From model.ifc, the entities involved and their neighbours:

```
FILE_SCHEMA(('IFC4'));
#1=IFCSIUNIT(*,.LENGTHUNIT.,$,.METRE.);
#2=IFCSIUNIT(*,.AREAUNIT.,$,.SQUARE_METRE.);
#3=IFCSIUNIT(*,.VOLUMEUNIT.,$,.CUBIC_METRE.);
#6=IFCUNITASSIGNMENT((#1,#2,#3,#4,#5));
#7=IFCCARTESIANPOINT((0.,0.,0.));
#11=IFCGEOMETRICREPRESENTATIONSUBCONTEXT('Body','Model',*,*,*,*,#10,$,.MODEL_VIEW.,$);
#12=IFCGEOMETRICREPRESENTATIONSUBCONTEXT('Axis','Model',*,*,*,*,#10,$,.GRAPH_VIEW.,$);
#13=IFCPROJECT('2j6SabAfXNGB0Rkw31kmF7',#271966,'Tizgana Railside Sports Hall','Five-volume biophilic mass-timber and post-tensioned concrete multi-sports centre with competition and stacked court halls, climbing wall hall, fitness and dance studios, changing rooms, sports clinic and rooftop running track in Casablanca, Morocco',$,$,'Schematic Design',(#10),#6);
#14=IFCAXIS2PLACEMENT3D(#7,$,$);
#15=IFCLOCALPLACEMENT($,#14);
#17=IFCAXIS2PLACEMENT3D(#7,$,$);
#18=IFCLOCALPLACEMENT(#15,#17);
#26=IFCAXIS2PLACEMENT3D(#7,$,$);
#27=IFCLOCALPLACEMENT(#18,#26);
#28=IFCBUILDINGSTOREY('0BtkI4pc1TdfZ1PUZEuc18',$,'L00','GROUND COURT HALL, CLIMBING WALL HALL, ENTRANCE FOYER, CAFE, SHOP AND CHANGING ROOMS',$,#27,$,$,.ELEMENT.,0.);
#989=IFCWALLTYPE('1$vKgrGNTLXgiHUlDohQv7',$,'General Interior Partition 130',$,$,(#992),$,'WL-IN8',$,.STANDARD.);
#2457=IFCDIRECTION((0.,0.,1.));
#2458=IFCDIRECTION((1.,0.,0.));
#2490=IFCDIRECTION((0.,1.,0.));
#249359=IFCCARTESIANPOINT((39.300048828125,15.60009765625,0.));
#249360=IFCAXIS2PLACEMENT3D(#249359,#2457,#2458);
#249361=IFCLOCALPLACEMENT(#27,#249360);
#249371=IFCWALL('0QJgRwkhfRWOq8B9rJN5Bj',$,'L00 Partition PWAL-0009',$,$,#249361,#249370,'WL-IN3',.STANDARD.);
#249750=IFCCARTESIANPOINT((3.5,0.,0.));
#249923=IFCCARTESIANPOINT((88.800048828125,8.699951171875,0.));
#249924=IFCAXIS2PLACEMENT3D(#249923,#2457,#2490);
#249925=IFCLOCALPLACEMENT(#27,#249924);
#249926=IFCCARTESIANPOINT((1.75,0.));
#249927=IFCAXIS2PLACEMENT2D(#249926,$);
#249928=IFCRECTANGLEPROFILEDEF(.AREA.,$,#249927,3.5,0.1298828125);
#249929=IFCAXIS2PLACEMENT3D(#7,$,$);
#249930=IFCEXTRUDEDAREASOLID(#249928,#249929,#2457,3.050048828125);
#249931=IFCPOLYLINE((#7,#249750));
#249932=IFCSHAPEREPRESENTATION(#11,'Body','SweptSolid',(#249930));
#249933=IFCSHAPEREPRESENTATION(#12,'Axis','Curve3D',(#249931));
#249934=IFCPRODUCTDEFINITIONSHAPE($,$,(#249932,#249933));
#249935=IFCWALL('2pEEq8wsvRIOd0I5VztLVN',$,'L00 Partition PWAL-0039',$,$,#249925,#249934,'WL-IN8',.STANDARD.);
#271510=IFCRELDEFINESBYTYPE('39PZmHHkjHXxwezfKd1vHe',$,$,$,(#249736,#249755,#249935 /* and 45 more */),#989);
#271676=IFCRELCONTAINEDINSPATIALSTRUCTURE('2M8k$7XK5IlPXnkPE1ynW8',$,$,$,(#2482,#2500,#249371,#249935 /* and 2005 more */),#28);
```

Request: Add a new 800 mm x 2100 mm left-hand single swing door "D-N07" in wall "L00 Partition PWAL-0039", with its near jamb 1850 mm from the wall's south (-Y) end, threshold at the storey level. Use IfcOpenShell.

```python
import numpy as np
import ifcopenshell
import ifcopenshell.api.feature
import ifcopenshell.api.geometry
import ifcopenshell.api.root
import ifcopenshell.api.spatial
import ifcopenshell.geom
import ifcopenshell.util.element
import ifcopenshell.util.placement
import ifcopenshell.util.representation
import ifcopenshell.util.shape
import ifcopenshell.util.unit

model = ifcopenshell.open("model.ifc")
unit_scale = ifcopenshell.util.unit.calculate_unit_scale(model)
settings = ifcopenshell.geom.settings()


def volume(element):
    """Net volume in cubic metres, openings subtracted."""
    shape = ifcopenshell.geom.create_shape(settings, element)
    return ifcopenshell.util.shape.get_volume(shape.geometry)


wall = model.by_guid("2pEEq8wsvRIOd0I5VztLVN")
storey = ifcopenshell.util.element.get_container(wall, ifc_class="IfcBuildingStorey")
context = ifcopenshell.util.representation.get_context(model, "Model", "Body", "MODEL_VIEW")
before = volume(wall)

width, height, from_end, sill = 0.8, 2.1, 1.85, 0.0  # metres

# The wall runs along its own X axis, and the end named is its -X end.
wall_shape = ifcopenshell.geom.create_shape(settings, wall)
x, y, z = ifcopenshell.util.shape.get_vertices(wall_shape.geometry).T
start = x.min() + from_end
face, thickness = float(y.min()), float(y.max() - y.min())
wall_matrix = ifcopenshell.util.placement.get_local_placement(wall.ObjectPlacement)
level = ifcopenshell.util.placement.get_local_placement(storey.ObjectPlacement)[2, 3]


def in_wall(x, y):
    """Placement at x, y metres in the wall's axes, at sill height."""
    matrix = wall_matrix.copy()
    matrix[:, 3] = wall_matrix @ np.array([x / unit_scale, y / unit_scale, 0.0, 1.0])
    matrix[2, 3] = level + sill / unit_scale
    return matrix


# Opening: a box that overshoots both wall faces by 50 mm.
opening = ifcopenshell.api.root.create_entity(model, ifc_class="IfcOpeningElement", predefined_type="OPENING")
box = ifcopenshell.api.geometry.add_wall_representation(
    model, context=context, length=width, height=height, thickness=thickness + 0.1
)
ifcopenshell.api.geometry.assign_representation(model, product=opening, representation=box)
ifcopenshell.api.geometry.edit_object_placement(model, product=opening, matrix=in_wall(start, face - 0.05), is_si=False)
ifcopenshell.api.feature.add_feature(model, feature=opening, element=wall)

door = ifcopenshell.api.root.create_entity(model, ifc_class="IfcDoor", name="D-N07", predefined_type="DOOR")
door.OverallWidth, door.OverallHeight = width / unit_scale, height / unit_scale
door.OperationType = "SINGLE_SWING_LEFT"
body = ifcopenshell.api.geometry.add_door_representation(
    model,
    context=context,
    overall_width=door.OverallWidth,
    overall_height=door.OverallHeight,
    operation_type="SINGLE_SWING_LEFT",
    lining_properties={"LiningDepth": thickness / unit_scale, "ThresholdDepth": thickness / unit_scale},
)
ifcopenshell.api.geometry.assign_representation(model, product=door, representation=body)
ifcopenshell.api.spatial.assign_container(model, products=[door], relating_structure=storey)
ifcopenshell.api.feature.add_filling(model, opening=opening, element=door)

# The lining spans the wall, so the door starts at the wall face.
ifcopenshell.api.geometry.edit_object_placement(model, product=door, matrix=in_wall(start, face), is_si=False)

after = volume(wall)

print(f"wall volume {before:.3f} -> {after:.3f} m3")

model.write("model_edited.ifc")
```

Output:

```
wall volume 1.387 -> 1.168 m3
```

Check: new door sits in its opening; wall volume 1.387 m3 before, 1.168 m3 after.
